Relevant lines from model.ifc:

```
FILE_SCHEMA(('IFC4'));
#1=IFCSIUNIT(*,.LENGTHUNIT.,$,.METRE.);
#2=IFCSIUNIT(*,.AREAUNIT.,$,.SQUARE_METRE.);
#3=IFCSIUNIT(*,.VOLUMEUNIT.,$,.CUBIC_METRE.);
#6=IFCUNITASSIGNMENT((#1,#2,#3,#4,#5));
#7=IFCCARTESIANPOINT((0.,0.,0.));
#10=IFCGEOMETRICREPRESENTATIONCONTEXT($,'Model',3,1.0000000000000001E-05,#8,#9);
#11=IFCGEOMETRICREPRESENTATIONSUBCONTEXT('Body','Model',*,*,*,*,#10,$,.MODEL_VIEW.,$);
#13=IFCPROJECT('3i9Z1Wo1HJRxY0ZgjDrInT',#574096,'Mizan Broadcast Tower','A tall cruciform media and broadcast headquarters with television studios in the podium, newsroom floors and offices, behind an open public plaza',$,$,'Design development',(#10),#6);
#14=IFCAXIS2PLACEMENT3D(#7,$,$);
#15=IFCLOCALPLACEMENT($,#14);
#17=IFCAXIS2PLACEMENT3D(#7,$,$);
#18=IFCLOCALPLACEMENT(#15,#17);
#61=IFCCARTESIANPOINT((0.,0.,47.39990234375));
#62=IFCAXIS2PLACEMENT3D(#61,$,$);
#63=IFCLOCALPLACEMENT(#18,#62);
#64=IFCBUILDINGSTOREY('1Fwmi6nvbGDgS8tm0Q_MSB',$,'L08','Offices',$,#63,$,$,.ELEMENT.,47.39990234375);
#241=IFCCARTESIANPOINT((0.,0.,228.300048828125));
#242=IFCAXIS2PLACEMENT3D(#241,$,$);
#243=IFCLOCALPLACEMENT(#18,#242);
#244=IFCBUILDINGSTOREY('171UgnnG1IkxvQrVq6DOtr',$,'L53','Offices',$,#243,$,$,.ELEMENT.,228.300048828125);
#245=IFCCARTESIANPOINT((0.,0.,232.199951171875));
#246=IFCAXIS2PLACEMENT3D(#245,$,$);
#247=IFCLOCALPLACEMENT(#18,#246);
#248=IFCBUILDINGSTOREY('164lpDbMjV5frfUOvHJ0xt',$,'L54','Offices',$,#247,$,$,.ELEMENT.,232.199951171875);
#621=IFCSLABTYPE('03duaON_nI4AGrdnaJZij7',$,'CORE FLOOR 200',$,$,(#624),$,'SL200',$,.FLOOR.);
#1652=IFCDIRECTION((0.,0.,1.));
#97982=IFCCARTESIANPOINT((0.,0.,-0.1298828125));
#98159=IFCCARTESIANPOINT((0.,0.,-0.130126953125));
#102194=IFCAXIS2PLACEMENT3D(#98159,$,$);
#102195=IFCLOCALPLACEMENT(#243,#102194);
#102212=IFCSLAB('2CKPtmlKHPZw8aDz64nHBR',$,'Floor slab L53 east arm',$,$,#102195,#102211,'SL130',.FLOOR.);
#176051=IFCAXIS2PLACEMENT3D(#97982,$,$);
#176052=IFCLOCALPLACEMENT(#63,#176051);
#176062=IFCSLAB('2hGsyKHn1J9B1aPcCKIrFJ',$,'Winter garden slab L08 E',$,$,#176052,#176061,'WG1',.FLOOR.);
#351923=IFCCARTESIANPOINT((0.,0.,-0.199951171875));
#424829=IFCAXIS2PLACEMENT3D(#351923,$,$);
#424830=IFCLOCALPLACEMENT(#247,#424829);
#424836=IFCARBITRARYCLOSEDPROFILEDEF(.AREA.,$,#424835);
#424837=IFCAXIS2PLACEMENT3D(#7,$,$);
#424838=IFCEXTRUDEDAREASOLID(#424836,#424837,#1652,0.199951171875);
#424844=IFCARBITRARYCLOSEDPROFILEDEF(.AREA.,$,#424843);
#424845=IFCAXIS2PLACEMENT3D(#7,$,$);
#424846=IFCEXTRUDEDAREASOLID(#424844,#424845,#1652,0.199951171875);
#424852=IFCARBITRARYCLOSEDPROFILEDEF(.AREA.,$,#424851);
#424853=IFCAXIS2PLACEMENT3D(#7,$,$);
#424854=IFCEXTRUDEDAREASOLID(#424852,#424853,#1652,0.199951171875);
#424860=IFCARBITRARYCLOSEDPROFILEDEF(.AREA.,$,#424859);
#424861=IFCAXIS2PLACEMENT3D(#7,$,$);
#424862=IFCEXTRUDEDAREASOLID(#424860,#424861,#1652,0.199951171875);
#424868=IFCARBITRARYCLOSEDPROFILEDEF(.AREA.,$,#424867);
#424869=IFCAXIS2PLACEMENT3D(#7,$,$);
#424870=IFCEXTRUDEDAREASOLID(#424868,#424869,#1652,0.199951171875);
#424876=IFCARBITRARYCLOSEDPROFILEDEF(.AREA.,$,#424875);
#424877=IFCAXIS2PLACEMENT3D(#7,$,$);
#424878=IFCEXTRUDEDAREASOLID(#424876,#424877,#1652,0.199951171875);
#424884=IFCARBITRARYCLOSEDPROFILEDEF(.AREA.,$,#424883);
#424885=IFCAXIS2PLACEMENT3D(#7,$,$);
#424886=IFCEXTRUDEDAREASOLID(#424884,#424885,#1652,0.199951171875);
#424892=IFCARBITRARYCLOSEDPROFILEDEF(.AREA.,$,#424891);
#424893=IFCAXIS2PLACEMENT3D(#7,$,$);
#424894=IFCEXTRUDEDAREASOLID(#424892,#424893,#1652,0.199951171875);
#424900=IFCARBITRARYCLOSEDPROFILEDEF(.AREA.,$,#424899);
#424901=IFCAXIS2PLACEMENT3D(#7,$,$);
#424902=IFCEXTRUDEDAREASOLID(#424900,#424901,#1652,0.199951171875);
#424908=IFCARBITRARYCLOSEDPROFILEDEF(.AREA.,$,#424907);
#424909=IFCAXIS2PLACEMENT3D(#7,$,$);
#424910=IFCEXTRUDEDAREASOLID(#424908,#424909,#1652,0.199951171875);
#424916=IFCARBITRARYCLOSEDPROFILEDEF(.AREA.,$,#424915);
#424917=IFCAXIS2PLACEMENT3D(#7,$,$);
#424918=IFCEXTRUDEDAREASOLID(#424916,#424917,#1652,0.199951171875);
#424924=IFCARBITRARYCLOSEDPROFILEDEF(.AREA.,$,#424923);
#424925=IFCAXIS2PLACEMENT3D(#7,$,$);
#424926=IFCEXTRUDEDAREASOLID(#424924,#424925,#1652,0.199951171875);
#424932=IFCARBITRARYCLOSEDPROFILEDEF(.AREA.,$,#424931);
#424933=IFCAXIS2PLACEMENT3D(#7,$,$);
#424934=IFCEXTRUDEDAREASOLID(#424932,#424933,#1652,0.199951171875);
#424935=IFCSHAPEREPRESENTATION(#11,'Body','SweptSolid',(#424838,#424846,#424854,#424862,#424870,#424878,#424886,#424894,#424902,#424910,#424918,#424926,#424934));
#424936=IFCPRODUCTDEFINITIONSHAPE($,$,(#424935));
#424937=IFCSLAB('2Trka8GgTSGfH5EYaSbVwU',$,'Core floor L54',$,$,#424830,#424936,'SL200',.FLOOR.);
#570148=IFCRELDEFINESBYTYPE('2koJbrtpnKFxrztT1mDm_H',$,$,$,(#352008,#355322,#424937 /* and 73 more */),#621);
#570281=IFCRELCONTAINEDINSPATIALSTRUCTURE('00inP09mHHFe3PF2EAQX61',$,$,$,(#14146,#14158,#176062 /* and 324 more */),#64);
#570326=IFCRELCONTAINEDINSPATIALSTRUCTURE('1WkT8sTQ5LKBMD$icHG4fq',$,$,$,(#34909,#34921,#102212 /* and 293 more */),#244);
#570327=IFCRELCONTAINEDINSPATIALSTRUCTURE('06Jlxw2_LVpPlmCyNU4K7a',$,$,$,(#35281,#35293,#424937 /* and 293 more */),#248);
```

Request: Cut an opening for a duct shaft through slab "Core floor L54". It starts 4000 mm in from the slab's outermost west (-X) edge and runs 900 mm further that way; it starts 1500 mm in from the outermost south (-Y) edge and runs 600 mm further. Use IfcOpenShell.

```python
import numpy as np
import ifcopenshell
import ifcopenshell.api.feature
import ifcopenshell.api.geometry
import ifcopenshell.api.root
import ifcopenshell.geom
import ifcopenshell.util.placement
import ifcopenshell.util.representation
import ifcopenshell.util.shape
import ifcopenshell.util.unit

model = ifcopenshell.open("model.ifc")
unit_scale = ifcopenshell.util.unit.calculate_unit_scale(model)
settings = ifcopenshell.geom.settings()


def volume(element):
    """Net volume in cubic metres, openings subtracted."""
    shape = ifcopenshell.geom.create_shape(settings, element)
    return ifcopenshell.util.shape.get_volume(shape.geometry)


slab = model.by_guid("2Trka8GgTSGfH5EYaSbVwU")
before = volume(slab)

# Extent in the slab's own axes, in metres. The edges named are its -X and -Y sides.
slab_shape = ifcopenshell.geom.create_shape(settings, slab)
vertices = ifcopenshell.util.shape.get_vertices(slab_shape.geometry)
x_min, y_min, bottom = vertices.min(axis=0)
top = vertices[:, 2].max()

opening = ifcopenshell.api.root.create_entity(model, ifc_class="IfcOpeningElement", name="Duct shaft opening", predefined_type="OPENING")
context = ifcopenshell.util.representation.get_context(model, "Model", "Body", "MODEL_VIEW")
width, depth = 0.9, 0.6
outline = [(0.0, 0.0), (width, 0.0), (width, depth), (0.0, depth), (0.0, 0.0)]
# Overshoot both faces by 50 mm so the cut is clean.
shape = ifcopenshell.api.geometry.add_slab_representation(
    model, context=context, depth=top - bottom + 0.1, polyline=outline
)
ifcopenshell.api.geometry.assign_representation(model, product=opening, representation=shape)

matrix = ifcopenshell.util.placement.get_local_placement(slab.ObjectPlacement)
matrix[:, 3] = matrix @ np.append(np.array([x_min + 4, y_min + 1.5, bottom - 0.05]) / unit_scale, 1.0)
ifcopenshell.api.geometry.edit_object_placement(model, product=opening, matrix=matrix, is_si=False)
ifcopenshell.api.feature.add_feature(model, feature=opening, element=slab)

after = volume(slab)

print(f"slab volume {before:.3f} -> {after:.3f} m3")

model.write("model_rev.ifc")
```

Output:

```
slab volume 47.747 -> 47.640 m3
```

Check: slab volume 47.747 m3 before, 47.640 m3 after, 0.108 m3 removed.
